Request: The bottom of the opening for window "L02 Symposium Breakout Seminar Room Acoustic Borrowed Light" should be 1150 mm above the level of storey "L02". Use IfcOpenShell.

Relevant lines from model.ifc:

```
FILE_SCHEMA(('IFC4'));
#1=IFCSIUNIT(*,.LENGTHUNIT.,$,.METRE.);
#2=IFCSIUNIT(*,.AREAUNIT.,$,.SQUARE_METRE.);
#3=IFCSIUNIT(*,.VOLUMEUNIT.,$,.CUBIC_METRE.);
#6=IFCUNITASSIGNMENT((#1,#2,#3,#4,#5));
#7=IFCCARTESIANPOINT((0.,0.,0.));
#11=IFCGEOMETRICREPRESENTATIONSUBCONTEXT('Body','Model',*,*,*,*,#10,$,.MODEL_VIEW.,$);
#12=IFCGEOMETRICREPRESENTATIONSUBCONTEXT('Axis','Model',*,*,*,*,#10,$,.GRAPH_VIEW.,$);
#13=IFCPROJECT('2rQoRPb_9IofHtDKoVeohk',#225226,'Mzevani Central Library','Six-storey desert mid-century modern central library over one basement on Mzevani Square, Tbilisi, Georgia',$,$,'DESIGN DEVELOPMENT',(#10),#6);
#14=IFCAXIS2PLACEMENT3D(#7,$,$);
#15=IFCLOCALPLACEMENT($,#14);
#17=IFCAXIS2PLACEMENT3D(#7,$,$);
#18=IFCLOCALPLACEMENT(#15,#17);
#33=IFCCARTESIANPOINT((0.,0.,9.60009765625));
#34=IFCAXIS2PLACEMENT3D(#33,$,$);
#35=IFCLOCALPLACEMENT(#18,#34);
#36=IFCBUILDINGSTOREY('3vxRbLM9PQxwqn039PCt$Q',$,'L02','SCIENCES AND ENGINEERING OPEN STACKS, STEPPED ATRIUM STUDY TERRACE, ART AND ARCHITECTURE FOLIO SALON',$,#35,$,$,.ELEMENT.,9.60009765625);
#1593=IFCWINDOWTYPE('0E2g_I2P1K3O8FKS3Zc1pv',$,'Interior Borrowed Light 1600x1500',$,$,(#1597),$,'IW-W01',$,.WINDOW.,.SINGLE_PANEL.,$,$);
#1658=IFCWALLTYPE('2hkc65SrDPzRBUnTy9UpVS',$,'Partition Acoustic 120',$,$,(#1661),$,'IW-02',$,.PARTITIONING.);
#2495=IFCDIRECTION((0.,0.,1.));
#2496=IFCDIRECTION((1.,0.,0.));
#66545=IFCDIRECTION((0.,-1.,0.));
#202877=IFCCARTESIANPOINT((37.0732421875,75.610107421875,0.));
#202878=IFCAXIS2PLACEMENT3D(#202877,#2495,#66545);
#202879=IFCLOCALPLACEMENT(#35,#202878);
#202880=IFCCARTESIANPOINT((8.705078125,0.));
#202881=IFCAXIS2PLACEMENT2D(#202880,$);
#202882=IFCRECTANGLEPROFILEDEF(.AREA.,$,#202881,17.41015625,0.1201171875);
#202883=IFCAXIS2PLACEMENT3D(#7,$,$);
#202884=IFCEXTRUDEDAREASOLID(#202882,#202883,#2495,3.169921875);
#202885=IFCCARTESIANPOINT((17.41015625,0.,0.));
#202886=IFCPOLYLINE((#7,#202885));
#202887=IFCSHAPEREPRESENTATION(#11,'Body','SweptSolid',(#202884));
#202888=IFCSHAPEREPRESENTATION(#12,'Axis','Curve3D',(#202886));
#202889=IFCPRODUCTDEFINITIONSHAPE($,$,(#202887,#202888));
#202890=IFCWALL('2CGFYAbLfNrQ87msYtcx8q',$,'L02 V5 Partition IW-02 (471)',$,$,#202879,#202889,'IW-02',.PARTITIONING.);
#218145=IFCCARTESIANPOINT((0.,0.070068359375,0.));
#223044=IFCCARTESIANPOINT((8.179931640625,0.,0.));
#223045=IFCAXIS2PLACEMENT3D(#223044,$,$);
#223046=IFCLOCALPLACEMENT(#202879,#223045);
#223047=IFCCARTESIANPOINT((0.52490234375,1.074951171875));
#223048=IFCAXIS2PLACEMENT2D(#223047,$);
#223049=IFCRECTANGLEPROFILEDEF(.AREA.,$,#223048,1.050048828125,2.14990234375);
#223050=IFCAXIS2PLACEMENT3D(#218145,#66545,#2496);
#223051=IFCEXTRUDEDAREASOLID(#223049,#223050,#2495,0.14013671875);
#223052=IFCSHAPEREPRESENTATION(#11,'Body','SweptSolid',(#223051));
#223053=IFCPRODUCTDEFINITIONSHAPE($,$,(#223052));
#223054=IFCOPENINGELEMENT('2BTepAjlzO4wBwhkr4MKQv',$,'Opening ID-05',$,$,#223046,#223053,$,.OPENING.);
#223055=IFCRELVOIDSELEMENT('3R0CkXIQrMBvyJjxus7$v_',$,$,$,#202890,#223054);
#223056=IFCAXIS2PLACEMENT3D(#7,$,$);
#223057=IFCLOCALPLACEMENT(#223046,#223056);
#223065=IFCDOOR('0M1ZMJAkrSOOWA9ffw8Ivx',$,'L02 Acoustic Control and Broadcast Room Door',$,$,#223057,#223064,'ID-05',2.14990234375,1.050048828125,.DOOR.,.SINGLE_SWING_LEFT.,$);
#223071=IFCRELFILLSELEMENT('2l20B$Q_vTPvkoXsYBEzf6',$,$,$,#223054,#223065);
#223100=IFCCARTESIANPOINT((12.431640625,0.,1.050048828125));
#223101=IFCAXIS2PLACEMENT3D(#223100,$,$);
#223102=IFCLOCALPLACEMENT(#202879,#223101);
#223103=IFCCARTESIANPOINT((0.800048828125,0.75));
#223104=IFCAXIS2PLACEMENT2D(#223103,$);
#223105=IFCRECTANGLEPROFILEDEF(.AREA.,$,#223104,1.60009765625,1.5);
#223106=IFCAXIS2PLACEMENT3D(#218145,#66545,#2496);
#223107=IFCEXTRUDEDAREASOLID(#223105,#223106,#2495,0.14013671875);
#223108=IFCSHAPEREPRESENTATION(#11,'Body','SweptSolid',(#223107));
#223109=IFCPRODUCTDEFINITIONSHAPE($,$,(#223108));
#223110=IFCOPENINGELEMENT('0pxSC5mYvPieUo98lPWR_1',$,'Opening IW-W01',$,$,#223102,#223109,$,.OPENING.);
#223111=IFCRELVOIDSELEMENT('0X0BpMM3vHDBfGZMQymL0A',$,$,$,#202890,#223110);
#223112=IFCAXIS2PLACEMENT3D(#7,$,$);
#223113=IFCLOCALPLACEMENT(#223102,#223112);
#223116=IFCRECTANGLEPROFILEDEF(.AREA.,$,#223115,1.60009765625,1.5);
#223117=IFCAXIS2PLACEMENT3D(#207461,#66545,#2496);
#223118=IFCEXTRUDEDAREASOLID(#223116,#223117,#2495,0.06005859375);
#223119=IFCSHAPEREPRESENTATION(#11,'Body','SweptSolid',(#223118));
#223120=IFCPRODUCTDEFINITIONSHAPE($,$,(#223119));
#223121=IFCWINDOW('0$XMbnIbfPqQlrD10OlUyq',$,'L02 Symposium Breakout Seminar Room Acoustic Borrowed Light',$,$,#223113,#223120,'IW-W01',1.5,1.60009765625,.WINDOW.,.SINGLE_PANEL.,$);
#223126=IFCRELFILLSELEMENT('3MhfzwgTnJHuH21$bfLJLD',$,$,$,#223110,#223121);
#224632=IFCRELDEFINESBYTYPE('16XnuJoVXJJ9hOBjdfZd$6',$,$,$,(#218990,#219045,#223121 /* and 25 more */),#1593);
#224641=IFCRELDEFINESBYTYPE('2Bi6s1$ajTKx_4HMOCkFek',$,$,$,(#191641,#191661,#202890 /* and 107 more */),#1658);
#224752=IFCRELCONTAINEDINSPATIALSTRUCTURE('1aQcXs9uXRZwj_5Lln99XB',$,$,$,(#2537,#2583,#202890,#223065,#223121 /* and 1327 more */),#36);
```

```python
import numpy as np
import ifcopenshell
import ifcopenshell.api.geometry
import ifcopenshell.geom
import ifcopenshell.util.element
import ifcopenshell.util.placement
import ifcopenshell.util.shape
import ifcopenshell.util.unit

model = ifcopenshell.open("model.ifc")
unit_scale = ifcopenshell.util.unit.calculate_unit_scale(model)

window = model.by_id(223121)
opening = window.FillsVoids[0].RelatingOpeningElement
storey = ifcopenshell.util.element.get_container(window, ifc_class="IfcBuildingStorey")
level = ifcopenshell.util.placement.get_local_placement(storey.ObjectPlacement)[2, 3]

# The opening's origin need not be at the sill, so measure its lowest point.
shape = ifcopenshell.geom.create_shape(ifcopenshell.geom.settings(), opening)
bottom = ifcopenshell.util.shape.get_shape_bottom_elevation(shape, shape.geometry) / unit_scale
dz = level + 1.15 / unit_scale - bottom

shift = np.array([0.0, 0.0, dz])
# The window is placed relative to its opening, so it follows when the opening moves.
matrix = ifcopenshell.util.placement.get_local_placement(opening.ObjectPlacement)
matrix[:3, 3] += shift
ifcopenshell.api.geometry.edit_object_placement(
    model, product=opening, matrix=matrix, is_si=False, should_transform_children=True
)

print(f"moved by {dz * unit_scale:+.3f} m")

model.write("model_edited.ifc")
```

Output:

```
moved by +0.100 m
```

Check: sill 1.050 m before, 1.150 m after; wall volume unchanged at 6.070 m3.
